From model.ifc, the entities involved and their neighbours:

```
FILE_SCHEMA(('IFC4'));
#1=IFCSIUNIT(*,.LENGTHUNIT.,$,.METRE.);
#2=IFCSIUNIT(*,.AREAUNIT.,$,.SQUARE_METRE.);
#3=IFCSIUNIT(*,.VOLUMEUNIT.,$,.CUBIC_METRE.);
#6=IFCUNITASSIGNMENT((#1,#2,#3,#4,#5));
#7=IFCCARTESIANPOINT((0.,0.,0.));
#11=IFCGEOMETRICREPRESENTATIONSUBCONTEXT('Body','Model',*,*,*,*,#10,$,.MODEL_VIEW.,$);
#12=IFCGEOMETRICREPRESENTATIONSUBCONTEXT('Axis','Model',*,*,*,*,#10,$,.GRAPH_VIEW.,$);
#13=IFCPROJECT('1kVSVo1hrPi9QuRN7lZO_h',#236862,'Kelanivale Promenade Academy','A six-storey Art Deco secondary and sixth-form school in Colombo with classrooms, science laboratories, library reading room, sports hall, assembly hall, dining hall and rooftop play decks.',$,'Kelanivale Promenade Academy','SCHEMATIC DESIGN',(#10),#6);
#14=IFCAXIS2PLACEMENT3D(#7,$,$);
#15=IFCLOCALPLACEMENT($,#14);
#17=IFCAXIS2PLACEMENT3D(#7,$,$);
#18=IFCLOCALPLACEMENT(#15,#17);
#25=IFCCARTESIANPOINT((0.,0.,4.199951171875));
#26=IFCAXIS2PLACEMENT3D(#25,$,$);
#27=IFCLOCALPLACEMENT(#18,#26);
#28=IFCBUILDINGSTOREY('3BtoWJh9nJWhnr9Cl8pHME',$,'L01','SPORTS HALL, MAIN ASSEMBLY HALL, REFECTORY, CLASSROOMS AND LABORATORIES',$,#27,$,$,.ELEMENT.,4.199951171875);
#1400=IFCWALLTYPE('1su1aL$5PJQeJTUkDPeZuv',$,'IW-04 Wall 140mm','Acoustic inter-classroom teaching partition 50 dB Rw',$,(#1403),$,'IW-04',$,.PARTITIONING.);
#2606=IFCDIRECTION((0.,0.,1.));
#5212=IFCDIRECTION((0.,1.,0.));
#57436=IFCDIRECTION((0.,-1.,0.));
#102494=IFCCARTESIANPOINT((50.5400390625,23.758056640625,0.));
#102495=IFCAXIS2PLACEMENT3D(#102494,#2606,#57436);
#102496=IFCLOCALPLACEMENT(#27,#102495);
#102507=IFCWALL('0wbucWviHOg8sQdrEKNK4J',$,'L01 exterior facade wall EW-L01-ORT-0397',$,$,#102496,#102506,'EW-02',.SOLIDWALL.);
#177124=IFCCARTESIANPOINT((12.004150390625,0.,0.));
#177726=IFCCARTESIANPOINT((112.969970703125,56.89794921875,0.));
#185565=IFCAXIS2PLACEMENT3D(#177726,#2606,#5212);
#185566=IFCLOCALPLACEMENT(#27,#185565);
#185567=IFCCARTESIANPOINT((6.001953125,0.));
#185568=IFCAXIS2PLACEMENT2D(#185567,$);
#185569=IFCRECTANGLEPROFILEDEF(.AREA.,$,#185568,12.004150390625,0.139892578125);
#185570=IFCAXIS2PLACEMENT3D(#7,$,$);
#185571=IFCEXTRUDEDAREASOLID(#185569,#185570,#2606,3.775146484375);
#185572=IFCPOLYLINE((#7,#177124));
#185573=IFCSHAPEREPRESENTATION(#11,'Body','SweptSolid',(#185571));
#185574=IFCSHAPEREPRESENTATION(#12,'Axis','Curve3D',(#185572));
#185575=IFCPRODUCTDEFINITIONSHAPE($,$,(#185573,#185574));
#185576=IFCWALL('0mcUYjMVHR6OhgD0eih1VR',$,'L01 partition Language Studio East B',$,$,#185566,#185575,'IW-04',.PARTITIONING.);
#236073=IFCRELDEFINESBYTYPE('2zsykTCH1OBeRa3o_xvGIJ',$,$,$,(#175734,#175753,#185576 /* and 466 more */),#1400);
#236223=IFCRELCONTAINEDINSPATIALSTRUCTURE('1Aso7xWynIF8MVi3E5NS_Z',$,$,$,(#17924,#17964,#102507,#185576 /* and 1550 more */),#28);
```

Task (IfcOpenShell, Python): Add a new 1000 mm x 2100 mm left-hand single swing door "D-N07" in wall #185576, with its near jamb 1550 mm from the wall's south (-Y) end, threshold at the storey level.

```python
import numpy as np
import ifcopenshell
import ifcopenshell.api.feature
import ifcopenshell.api.geometry
import ifcopenshell.api.root
import ifcopenshell.api.spatial
import ifcopenshell.geom
import ifcopenshell.util.element
import ifcopenshell.util.placement
import ifcopenshell.util.representation
import ifcopenshell.util.shape
import ifcopenshell.util.unit

model = ifcopenshell.open("model.ifc")
unit_scale = ifcopenshell.util.unit.calculate_unit_scale(model)
settings = ifcopenshell.geom.settings()


def volume(element):
    """Net volume in cubic metres, openings subtracted."""
    shape = ifcopenshell.geom.create_shape(settings, element)
    return ifcopenshell.util.shape.get_volume(shape.geometry)


wall = model.by_id(185576)
storey = ifcopenshell.util.element.get_container(wall, ifc_class="IfcBuildingStorey")
context = ifcopenshell.util.representation.get_context(model, "Model", "Body", "MODEL_VIEW")
before = volume(wall)

width, height, from_end, sill = 1, 2.1, 1.55, 0.0  # metres

# The wall runs along its own X axis, and the end named is its -X end.
wall_shape = ifcopenshell.geom.create_shape(settings, wall)
x, y, z = ifcopenshell.util.shape.get_vertices(wall_shape.geometry).T
start = x.min() + from_end
face, thickness = float(y.min()), float(y.max() - y.min())
wall_matrix = ifcopenshell.util.placement.get_local_placement(wall.ObjectPlacement)
level = ifcopenshell.util.placement.get_local_placement(storey.ObjectPlacement)[2, 3]


def in_wall(x, y):
    """Placement at x, y metres in the wall's axes, at sill height."""
    matrix = wall_matrix.copy()
    matrix[:, 3] = wall_matrix @ np.array([x / unit_scale, y / unit_scale, 0.0, 1.0])
    matrix[2, 3] = level + sill / unit_scale
    return matrix


# Opening: a box that overshoots both wall faces by 50 mm.
opening = ifcopenshell.api.root.create_entity(model, ifc_class="IfcOpeningElement", predefined_type="OPENING")
box = ifcopenshell.api.geometry.add_wall_representation(
    model, context=context, length=width, height=height, thickness=thickness + 0.1
)
ifcopenshell.api.geometry.assign_representation(model, product=opening, representation=box)
ifcopenshell.api.geometry.edit_object_placement(model, product=opening, matrix=in_wall(start, face - 0.05), is_si=False)
ifcopenshell.api.feature.add_feature(model, feature=opening, element=wall)

door = ifcopenshell.api.root.create_entity(model, ifc_class="IfcDoor", name="D-N07", predefined_type="DOOR")
door.OverallWidth, door.OverallHeight = width / unit_scale, height / unit_scale
door.OperationType = "SINGLE_SWING_LEFT"
body = ifcopenshell.api.geometry.add_door_representation(
    model,
    context=context,
    overall_width=door.OverallWidth,
    overall_height=door.OverallHeight,
    operation_type="SINGLE_SWING_LEFT",
    lining_properties={"LiningDepth": thickness / unit_scale, "ThresholdDepth": thickness / unit_scale},
)
ifcopenshell.api.geometry.assign_representation(model, product=door, representation=body)
ifcopenshell.api.spatial.assign_container(model, products=[door], relating_structure=storey)
ifcopenshell.api.feature.add_filling(model, opening=opening, element=door)

# The lining spans the wall, so the door starts at the wall face.
ifcopenshell.api.geometry.edit_object_placement(model, product=door, matrix=in_wall(start, face), is_si=False)

after = volume(wall)

print(f"wall volume {before:.3f} -> {after:.3f} m3")

model.write("model_edited.ifc")
```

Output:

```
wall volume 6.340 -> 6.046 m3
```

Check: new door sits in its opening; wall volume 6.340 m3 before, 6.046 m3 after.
